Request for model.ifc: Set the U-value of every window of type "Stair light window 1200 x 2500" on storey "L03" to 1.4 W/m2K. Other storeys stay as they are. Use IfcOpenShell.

First a look at what the model holds.

```python
import ifcopenshell
import ifcopenshell.util.element

model = ifcopenshell.open("model.ifc")
print(model.schema)
storey = next(s for s in model.by_type("IfcBuildingStorey") if s.Name == "L03")
windows = [e for e in ifcopenshell.util.element.get_decomposition(storey) if e.is_a("IfcWindow")]
seen = {}
for e in windows:
    element_type = ifcopenshell.util.element.get_type(e)
    key = (element_type.Name if element_type != e and element_type else None, ifcopenshell.util.element.get_pset(e, "Pset_WindowCommon", "ThermalTransmittance"))
    seen[key] = seen.get(key, 0) + 1
for (name, value), count in sorted(seen.items(), key=str):
    print(count, "x", name, "|", value)
```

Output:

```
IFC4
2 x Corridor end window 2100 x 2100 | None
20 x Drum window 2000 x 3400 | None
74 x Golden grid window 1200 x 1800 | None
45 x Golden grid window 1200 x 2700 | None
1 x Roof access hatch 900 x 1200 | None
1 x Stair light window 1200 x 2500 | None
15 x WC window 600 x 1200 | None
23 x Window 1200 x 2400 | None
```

```python
import ifcopenshell
import ifcopenshell.api.pset
import ifcopenshell.util.element

model = ifcopenshell.open("model.ifc")

storey = next(s for s in model.by_type("IfcBuildingStorey") if s.Name == "L03")
windows = [e for e in ifcopenshell.util.element.get_decomposition(storey) if e.is_a("IfcWindow")]

count = 0
for e in windows:
    element_type = ifcopenshell.util.element.get_type(e)
    if element_type in (None, e) or element_type.Name != "Stair light window 1200 x 2500":
        continue
    # add_pset returns the element's existing set when there is one.
    pset = ifcopenshell.api.pset.add_pset(model, product=e, name="Pset_WindowCommon")
    ifcopenshell.api.pset.edit_pset(model, pset=pset, properties={"ThermalTransmittance": 1.4})
    count += 1

print(count, "windows updated")

model.write("model-out.ifc")
```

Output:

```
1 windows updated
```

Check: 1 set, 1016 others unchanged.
